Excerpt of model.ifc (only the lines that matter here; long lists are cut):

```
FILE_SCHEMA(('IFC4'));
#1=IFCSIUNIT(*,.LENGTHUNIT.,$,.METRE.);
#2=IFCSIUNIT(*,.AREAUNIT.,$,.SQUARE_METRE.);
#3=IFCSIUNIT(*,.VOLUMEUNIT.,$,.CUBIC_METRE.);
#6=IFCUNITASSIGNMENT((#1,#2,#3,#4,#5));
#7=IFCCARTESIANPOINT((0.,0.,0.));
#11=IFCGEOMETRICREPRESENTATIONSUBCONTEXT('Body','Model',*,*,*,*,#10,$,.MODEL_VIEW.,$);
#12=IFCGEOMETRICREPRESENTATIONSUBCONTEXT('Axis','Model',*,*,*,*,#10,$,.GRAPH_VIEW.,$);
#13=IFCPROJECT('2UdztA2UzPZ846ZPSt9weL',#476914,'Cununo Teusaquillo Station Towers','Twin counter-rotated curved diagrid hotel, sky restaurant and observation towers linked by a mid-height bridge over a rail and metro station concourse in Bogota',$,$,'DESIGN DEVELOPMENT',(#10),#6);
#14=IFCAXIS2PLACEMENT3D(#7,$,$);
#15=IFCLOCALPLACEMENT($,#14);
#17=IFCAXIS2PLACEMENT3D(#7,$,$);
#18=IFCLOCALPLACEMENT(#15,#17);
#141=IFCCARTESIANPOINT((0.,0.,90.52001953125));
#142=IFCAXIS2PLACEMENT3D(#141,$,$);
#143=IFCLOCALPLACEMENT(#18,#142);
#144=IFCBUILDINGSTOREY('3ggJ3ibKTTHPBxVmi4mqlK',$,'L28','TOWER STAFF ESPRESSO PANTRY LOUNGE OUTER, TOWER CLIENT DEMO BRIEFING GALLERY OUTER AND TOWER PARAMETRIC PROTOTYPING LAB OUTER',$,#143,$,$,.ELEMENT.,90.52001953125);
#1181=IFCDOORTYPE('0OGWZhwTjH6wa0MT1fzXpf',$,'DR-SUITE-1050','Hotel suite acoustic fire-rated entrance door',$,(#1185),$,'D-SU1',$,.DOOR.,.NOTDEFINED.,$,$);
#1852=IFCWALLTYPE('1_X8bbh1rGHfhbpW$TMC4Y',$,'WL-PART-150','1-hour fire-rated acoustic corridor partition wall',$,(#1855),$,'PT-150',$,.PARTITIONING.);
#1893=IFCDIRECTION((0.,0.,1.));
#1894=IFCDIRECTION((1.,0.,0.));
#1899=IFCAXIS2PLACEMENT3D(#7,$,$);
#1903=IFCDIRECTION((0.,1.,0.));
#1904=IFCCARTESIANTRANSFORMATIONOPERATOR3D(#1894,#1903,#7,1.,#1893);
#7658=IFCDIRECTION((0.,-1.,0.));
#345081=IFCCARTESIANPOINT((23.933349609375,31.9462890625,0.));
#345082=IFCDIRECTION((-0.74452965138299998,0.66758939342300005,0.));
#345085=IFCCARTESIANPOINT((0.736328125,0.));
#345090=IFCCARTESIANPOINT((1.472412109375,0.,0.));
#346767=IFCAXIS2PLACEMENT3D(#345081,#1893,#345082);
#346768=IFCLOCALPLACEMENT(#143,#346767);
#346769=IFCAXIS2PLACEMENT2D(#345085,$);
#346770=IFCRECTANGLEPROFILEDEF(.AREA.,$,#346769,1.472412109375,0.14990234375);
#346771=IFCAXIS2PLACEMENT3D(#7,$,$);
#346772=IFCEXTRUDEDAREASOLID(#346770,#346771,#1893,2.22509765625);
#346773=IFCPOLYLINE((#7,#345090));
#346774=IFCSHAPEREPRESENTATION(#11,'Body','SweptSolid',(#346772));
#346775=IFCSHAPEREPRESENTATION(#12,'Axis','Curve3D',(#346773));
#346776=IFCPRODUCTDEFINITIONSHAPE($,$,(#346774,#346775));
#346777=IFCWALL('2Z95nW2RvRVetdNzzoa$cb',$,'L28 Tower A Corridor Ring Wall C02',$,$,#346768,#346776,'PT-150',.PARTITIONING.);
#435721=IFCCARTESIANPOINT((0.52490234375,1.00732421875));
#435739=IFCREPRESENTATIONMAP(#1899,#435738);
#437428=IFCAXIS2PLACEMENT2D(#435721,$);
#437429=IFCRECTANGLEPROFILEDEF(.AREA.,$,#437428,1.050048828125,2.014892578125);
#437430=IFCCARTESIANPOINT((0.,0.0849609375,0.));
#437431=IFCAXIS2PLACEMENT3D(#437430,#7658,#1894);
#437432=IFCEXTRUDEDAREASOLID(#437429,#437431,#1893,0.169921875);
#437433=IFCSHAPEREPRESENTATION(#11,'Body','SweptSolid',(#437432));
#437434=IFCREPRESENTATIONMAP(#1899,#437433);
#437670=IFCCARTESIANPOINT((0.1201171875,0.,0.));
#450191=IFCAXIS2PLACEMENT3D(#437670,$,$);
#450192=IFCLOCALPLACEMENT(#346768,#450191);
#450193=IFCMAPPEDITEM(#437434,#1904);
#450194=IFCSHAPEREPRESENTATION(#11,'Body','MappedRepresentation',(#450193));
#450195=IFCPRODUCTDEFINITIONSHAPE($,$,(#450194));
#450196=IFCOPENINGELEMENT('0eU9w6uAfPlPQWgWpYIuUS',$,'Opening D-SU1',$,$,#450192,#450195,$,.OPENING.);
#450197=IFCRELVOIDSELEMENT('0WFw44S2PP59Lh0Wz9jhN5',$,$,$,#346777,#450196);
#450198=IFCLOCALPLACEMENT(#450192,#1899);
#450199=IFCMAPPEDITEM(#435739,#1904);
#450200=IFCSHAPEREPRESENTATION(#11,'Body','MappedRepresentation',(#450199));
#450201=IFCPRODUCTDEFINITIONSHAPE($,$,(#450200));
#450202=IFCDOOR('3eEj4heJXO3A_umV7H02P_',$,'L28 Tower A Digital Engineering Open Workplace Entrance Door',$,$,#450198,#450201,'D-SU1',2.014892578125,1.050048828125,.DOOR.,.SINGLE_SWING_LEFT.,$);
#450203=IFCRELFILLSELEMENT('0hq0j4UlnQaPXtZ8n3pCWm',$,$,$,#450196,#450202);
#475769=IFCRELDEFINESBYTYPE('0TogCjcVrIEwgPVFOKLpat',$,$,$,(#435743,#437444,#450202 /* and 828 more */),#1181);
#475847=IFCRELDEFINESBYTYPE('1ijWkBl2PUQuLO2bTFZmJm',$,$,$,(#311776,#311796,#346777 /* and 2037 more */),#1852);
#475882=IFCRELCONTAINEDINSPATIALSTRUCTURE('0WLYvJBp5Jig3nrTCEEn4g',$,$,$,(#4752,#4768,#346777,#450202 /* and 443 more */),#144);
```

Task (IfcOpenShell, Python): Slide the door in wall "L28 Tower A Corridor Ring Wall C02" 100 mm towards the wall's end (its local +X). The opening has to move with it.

```python
import ifcopenshell
import ifcopenshell.api.geometry
import ifcopenshell.util.placement

model = ifcopenshell.open("model.ifc")

door = model.by_guid("3eEj4heJXO3A_umV7H02P_")
opening = door.FillsVoids[0].RelatingOpeningElement
wall = opening.VoidsElements[0].RelatingBuildingElement

wall_matrix = ifcopenshell.util.placement.get_local_placement(wall.ObjectPlacement)
shift = wall_matrix[:3, 0] * 0.1
before = ifcopenshell.util.placement.get_local_placement(door.ObjectPlacement)[:3, 3].copy()

# The door is placed relative to its opening, so it follows when the opening moves.
matrix = ifcopenshell.util.placement.get_local_placement(opening.ObjectPlacement)
matrix[:3, 3] += shift
ifcopenshell.api.geometry.edit_object_placement(
    model, product=opening, matrix=matrix, is_si=False, should_transform_children=True
)

after = ifcopenshell.util.placement.get_local_placement(door.ObjectPlacement)[:3, 3]
print("door moved by", (after - before).round(3) + 0.0)

model.write("model_updated.ifc")
```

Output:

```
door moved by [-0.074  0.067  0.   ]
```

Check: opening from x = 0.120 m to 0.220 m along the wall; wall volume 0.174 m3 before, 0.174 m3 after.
